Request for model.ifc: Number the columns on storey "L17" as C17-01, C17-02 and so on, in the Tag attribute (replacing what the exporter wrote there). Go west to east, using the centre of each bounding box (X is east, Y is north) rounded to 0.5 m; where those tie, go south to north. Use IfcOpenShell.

First a look at what the model holds.

```python
import ifcopenshell
import ifcopenshell.util.element
import ifcopenshell.util.placement

model = ifcopenshell.open("model.ifc")
print(model.schema)
storey = next(s for s in model.by_type("IfcBuildingStorey") if s.Name == "L17")
columns = [e for e in ifcopenshell.util.element.get_decomposition(storey) if e.is_a("IfcColumn")]
for e in sorted(columns, key=lambda e: e.id()):
    origin = ifcopenshell.util.placement.get_local_placement(e.ObjectPlacement)[:3, 3]
    print(e.id(), e.Tag, e.Name, origin.round(2) + 0.0, sep=" | ")
```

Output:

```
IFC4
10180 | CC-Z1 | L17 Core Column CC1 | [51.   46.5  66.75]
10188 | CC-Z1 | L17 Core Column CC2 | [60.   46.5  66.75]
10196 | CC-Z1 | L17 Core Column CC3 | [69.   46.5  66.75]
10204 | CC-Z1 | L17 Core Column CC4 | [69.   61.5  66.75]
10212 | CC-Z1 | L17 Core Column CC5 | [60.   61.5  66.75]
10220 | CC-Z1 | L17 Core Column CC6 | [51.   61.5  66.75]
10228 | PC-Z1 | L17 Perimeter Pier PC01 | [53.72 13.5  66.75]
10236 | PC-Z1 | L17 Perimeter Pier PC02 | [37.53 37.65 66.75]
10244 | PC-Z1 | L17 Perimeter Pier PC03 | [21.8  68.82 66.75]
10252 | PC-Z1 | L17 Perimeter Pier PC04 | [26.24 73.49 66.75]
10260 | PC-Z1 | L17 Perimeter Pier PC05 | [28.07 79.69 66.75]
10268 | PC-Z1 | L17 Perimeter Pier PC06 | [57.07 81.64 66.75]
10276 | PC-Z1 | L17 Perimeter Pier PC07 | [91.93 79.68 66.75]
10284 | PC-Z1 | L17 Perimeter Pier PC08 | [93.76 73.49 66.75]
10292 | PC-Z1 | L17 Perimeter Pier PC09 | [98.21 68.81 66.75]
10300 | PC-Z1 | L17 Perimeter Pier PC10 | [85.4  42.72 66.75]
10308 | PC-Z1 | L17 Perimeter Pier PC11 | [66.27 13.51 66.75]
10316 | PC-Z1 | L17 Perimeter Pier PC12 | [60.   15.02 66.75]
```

```python
import ifcopenshell
import ifcopenshell.geom
import ifcopenshell.util.element
import ifcopenshell.util.shape

model = ifcopenshell.open("model.ifc")
settings = ifcopenshell.geom.settings()
settings.set("use-world-coords", True)


def centre(element):
    shape = ifcopenshell.geom.create_shape(settings, element)
    return ifcopenshell.util.shape.get_bbox_centroid(shape.geometry)


storey = next(s for s in model.by_type("IfcBuildingStorey") if s.Name == "L17")
columns = [e for e in ifcopenshell.util.element.get_decomposition(storey) if e.is_a("IfcColumn")]

# Insertion points can sit at a corner or the storey origin, so sort by the geometry (in metres).
centres = {e: centre(e) for e in columns}
columns.sort(key=lambda e: (round(centres[e][0] / 0.5), centres[e][1]))

for i, e in enumerate(columns, start=1):
    number = f"C17-{i:02d}"
    e.Tag = number
    print(e.id(), number)

model.write("model_edited.ifc")
```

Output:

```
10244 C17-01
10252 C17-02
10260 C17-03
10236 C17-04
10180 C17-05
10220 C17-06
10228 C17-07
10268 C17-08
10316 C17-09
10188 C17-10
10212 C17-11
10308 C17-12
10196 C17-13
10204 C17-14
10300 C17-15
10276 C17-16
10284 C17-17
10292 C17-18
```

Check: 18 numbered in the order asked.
